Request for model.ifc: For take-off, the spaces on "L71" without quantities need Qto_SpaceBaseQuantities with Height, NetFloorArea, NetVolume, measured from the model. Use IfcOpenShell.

First a look at what the model holds.

```python
import ifcopenshell
import ifcopenshell.util.element
import ifcopenshell.util.unit

model = ifcopenshell.open("model.ifc")
print(model.schema)
for unit_type in ("LENGTHUNIT", "AREAUNIT", "VOLUMEUNIT"):
    print(unit_type, ifcopenshell.util.unit.calculate_unit_scale(model, unit_type))
storey = next(s for s in model.by_type("IfcBuildingStorey") if s.Name == "L71")
spaces = [e for e in ifcopenshell.util.element.get_decomposition(storey) if e.is_a("IfcSpace")]
for e in sorted(spaces, key=lambda e: e.id()):
    print(e.id(), e.is_a(), e.Name, list(ifcopenshell.util.element.get_psets(e, qtos_only=True)), sep=" | ")
```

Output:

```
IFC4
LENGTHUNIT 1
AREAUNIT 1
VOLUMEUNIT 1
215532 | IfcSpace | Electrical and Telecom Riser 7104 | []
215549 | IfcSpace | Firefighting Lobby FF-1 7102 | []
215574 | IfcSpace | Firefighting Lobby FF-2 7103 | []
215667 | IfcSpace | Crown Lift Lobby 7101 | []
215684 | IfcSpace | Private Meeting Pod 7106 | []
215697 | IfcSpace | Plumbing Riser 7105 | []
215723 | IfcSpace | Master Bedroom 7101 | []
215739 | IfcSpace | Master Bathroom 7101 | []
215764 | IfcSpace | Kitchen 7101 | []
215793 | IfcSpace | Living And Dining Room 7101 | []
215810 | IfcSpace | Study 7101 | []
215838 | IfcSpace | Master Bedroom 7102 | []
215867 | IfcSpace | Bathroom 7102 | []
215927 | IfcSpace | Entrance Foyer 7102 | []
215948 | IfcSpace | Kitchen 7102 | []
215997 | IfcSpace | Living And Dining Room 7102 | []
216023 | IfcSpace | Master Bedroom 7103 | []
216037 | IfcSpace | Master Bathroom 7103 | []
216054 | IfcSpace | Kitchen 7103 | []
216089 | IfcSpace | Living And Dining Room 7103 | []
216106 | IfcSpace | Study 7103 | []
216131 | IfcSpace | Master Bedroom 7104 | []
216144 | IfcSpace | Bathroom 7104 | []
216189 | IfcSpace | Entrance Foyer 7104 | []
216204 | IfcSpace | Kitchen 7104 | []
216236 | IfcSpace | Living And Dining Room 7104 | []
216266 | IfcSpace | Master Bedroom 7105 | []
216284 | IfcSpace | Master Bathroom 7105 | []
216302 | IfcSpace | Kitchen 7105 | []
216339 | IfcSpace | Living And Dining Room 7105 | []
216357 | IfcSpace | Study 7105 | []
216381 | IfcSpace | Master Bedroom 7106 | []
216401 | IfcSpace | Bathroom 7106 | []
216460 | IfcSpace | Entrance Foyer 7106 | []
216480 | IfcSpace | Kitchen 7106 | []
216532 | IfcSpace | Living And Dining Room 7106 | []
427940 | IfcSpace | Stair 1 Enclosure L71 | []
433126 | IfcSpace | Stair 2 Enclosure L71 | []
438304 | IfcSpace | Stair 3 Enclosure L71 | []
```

```python
import ifcopenshell
import ifcopenshell.api.pset
import ifcopenshell.geom
import ifcopenshell.util.element
import ifcopenshell.util.shape
import ifcopenshell.util.unit

model = ifcopenshell.open("model.ifc")
unit_scale = ifcopenshell.util.unit.calculate_unit_scale(model)
area_scale = ifcopenshell.util.unit.calculate_unit_scale(model, "AREAUNIT")
volume_scale = ifcopenshell.util.unit.calculate_unit_scale(model, "VOLUMEUNIT")
settings = ifcopenshell.geom.settings()

storey = next(s for s in model.by_type("IfcBuildingStorey") if s.Name == "L71")
spaces = [e for e in ifcopenshell.util.element.get_decomposition(storey) if e.is_a("IfcSpace")]

for e in sorted(spaces, key=lambda e: e.id()):
    if ifcopenshell.util.element.get_psets(e, qtos_only=True, should_inherit=False):
        continue
    # Geometry comes back in metres, in the element's own axes.
    shape = ifcopenshell.geom.create_shape(settings, e)
    values = {
        "Height": ifcopenshell.util.shape.get_z(shape.geometry) / unit_scale,
        "NetFloorArea": ifcopenshell.util.shape.get_footprint_area(shape.geometry) / area_scale,
        "NetVolume": ifcopenshell.util.shape.get_volume(shape.geometry) / volume_scale,
    }
    qto = ifcopenshell.api.pset.add_qto(model, product=e, name="Qto_SpaceBaseQuantities")
    ifcopenshell.api.pset.edit_qto(model, qto=qto, properties=values)
    print(e.id(), {k: round(v, 3) for k, v in values.items()})

model.write("model-out.ifc")
```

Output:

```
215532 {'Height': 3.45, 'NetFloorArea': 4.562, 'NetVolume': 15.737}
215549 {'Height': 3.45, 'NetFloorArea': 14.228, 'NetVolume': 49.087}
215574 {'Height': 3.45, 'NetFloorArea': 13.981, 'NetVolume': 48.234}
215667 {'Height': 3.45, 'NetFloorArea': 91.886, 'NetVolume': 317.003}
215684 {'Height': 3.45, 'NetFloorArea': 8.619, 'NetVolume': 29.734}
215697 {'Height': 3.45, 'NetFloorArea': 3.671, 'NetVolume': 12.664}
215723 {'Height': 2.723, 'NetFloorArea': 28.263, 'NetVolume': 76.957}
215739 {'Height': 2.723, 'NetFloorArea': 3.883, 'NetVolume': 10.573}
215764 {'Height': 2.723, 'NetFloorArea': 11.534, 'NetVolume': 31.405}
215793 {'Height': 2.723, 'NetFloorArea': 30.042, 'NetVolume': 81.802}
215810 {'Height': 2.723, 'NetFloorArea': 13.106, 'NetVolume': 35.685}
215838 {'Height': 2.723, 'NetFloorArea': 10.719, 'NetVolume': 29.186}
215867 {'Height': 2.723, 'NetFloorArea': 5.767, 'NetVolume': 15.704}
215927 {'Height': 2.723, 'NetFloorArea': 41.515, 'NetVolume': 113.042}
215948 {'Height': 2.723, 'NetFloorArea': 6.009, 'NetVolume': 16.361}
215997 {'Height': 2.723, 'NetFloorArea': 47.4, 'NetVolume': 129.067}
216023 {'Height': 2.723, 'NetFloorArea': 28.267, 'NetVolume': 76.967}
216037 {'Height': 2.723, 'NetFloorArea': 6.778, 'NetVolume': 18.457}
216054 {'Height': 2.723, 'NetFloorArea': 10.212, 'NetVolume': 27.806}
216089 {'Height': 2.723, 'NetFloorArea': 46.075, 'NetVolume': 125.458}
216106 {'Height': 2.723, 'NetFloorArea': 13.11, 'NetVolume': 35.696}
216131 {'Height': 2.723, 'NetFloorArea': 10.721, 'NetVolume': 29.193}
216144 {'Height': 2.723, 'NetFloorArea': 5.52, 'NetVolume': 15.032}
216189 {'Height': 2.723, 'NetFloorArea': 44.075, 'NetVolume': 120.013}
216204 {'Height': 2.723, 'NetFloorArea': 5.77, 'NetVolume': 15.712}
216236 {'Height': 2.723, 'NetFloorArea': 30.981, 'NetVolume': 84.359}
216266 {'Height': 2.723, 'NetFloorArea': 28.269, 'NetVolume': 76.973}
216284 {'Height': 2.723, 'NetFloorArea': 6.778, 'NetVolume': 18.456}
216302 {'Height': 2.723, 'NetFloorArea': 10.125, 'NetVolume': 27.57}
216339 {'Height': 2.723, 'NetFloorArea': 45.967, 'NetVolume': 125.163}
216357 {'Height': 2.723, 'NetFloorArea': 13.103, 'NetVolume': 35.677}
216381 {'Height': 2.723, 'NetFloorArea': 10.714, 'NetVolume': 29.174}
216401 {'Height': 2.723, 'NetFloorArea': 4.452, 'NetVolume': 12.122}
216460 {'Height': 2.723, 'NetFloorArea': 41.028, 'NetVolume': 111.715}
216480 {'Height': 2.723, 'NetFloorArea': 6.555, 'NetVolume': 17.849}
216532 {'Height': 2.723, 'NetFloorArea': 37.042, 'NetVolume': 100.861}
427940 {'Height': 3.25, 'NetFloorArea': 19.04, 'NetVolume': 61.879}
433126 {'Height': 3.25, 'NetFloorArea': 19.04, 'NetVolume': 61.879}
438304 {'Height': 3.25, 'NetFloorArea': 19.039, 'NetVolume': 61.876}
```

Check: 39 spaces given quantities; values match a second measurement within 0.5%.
